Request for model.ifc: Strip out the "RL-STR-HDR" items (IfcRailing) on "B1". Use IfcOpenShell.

First a look at what the model holds.

```python
import ifcopenshell
import ifcopenshell.util.element

model = ifcopenshell.open("model.ifc")
print(model.schema)
storey = next(s for s in model.by_type("IfcBuildingStorey") if s.Name == "B1")
railings = [e for e in ifcopenshell.util.element.get_decomposition(storey) if e.is_a("IfcRailing")]
seen = {}
for e in railings:
    element_type = ifcopenshell.util.element.get_type(e)
    name = element_type.Name if element_type not in (None, e) else None
    seen[name] = seen.get(name, 0) + 1
for name, count in sorted(seen.items(), key=str):
    print(count, "x", name)
```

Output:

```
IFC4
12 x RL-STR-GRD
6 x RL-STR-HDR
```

```python
import ifcopenshell
import ifcopenshell.api.root
import ifcopenshell.util.element

model = ifcopenshell.open("model.ifc")

storey = next(s for s in model.by_type("IfcBuildingStorey") if s.Name == "B1")
railings = [e for e in ifcopenshell.util.element.get_decomposition(storey) if e.is_a("IfcRailing")]
targets = [e for e in railings if (t := ifcopenshell.util.element.get_type(e)) not in (None, e) and t.Name == "RL-STR-HDR"]

for e in targets:
    ifcopenshell.api.root.remove_product(model, product=e)
print(len(targets), "removed")

model.write("model_v2.ifc")
```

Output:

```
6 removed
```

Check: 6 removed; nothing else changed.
